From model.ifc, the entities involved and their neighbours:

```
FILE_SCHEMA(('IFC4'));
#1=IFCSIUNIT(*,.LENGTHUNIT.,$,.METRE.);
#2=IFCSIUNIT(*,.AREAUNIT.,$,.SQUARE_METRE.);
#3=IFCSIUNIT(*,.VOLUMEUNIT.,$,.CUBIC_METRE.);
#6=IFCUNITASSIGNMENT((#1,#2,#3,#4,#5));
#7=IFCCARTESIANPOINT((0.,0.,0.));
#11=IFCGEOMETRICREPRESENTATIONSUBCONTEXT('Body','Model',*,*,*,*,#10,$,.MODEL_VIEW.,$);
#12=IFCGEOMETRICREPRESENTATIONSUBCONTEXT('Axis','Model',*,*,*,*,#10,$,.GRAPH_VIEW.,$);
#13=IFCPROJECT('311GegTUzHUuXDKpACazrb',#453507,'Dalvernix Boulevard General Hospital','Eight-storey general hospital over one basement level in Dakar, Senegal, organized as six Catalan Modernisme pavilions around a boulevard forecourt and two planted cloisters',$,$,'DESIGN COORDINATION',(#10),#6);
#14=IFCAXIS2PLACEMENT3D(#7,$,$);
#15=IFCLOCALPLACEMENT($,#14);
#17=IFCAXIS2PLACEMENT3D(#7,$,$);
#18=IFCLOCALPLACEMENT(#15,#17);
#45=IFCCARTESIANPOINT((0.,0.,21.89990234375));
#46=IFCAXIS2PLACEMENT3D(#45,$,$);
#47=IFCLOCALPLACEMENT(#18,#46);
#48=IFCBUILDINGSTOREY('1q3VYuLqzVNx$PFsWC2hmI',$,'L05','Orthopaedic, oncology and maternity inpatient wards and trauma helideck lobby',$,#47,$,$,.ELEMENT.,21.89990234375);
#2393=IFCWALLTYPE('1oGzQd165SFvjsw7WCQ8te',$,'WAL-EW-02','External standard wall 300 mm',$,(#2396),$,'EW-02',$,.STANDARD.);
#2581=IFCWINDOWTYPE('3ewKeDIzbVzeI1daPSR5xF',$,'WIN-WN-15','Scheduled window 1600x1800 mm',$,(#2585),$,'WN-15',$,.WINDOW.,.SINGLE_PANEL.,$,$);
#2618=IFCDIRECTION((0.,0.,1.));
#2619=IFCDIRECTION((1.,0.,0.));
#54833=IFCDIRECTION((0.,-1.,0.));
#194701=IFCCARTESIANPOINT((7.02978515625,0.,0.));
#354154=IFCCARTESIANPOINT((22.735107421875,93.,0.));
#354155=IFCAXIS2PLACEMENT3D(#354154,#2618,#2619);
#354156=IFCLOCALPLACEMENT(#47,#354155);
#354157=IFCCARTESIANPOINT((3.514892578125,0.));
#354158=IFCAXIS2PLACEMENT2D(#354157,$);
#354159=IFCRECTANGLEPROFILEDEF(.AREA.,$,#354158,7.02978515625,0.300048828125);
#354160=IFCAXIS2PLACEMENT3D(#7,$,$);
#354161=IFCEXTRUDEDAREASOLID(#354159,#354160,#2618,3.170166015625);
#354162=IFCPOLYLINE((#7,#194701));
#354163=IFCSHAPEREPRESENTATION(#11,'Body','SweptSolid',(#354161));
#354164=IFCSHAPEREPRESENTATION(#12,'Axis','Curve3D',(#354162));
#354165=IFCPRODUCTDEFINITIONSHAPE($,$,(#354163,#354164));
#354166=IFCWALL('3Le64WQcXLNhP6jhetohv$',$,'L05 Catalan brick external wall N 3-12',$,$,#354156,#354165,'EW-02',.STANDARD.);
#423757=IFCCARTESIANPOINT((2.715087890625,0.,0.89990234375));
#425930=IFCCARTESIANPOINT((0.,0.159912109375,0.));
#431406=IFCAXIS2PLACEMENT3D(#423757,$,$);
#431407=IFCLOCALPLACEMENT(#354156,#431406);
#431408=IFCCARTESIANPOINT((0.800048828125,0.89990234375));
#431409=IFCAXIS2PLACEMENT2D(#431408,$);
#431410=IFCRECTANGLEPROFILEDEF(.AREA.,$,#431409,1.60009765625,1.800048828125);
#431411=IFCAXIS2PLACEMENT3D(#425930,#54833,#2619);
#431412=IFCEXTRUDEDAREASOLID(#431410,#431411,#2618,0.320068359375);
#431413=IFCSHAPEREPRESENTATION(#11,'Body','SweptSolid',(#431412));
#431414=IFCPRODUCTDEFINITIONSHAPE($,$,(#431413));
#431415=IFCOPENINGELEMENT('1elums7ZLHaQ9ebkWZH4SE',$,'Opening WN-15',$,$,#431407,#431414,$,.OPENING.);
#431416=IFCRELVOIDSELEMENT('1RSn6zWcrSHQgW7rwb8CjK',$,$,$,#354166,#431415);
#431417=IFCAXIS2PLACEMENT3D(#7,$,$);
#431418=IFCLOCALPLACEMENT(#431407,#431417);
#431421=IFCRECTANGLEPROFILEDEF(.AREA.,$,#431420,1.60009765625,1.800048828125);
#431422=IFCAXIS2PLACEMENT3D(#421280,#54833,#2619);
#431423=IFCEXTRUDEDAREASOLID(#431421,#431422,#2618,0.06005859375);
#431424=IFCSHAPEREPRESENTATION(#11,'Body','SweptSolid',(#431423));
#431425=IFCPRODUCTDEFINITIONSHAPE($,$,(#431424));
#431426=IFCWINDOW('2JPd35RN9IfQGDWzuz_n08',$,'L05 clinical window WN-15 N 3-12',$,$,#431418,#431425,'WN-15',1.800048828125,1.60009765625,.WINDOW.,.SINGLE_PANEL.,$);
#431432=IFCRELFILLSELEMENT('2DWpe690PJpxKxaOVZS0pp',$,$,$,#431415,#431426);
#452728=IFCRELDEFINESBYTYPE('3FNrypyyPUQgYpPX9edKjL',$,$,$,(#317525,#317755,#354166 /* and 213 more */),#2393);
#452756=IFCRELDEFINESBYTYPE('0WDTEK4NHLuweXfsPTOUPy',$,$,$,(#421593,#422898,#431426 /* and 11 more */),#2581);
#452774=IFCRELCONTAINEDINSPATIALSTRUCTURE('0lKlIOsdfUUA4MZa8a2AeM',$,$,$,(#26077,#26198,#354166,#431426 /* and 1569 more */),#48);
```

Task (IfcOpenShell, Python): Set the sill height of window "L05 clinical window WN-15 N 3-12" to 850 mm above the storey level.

```python
import numpy as np
import ifcopenshell
import ifcopenshell.api.geometry
import ifcopenshell.geom
import ifcopenshell.util.element
import ifcopenshell.util.placement
import ifcopenshell.util.shape
import ifcopenshell.util.unit

model = ifcopenshell.open("model.ifc")
unit_scale = ifcopenshell.util.unit.calculate_unit_scale(model)

window = model.by_guid("2JPd35RN9IfQGDWzuz_n08")
opening = window.FillsVoids[0].RelatingOpeningElement
storey = ifcopenshell.util.element.get_container(window, ifc_class="IfcBuildingStorey")
level = ifcopenshell.util.placement.get_local_placement(storey.ObjectPlacement)[2, 3]

# The opening's origin need not be at the sill, so measure its lowest point.
shape = ifcopenshell.geom.create_shape(ifcopenshell.geom.settings(), opening)
bottom = ifcopenshell.util.shape.get_shape_bottom_elevation(shape, shape.geometry) / unit_scale
dz = level + 0.85 - bottom

shift = np.array([0.0, 0.0, dz])
# The window is placed relative to its opening, so it follows when the opening moves.
matrix = ifcopenshell.util.placement.get_local_placement(opening.ObjectPlacement)
matrix[:3, 3] += shift
ifcopenshell.api.geometry.edit_object_placement(
    model, product=opening, matrix=matrix, is_si=False, should_transform_children=True
)

print(f"moved by {dz * unit_scale:+.3f} m")

model.write("model_rev.ifc")
```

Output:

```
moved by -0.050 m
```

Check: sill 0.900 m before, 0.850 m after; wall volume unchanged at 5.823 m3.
